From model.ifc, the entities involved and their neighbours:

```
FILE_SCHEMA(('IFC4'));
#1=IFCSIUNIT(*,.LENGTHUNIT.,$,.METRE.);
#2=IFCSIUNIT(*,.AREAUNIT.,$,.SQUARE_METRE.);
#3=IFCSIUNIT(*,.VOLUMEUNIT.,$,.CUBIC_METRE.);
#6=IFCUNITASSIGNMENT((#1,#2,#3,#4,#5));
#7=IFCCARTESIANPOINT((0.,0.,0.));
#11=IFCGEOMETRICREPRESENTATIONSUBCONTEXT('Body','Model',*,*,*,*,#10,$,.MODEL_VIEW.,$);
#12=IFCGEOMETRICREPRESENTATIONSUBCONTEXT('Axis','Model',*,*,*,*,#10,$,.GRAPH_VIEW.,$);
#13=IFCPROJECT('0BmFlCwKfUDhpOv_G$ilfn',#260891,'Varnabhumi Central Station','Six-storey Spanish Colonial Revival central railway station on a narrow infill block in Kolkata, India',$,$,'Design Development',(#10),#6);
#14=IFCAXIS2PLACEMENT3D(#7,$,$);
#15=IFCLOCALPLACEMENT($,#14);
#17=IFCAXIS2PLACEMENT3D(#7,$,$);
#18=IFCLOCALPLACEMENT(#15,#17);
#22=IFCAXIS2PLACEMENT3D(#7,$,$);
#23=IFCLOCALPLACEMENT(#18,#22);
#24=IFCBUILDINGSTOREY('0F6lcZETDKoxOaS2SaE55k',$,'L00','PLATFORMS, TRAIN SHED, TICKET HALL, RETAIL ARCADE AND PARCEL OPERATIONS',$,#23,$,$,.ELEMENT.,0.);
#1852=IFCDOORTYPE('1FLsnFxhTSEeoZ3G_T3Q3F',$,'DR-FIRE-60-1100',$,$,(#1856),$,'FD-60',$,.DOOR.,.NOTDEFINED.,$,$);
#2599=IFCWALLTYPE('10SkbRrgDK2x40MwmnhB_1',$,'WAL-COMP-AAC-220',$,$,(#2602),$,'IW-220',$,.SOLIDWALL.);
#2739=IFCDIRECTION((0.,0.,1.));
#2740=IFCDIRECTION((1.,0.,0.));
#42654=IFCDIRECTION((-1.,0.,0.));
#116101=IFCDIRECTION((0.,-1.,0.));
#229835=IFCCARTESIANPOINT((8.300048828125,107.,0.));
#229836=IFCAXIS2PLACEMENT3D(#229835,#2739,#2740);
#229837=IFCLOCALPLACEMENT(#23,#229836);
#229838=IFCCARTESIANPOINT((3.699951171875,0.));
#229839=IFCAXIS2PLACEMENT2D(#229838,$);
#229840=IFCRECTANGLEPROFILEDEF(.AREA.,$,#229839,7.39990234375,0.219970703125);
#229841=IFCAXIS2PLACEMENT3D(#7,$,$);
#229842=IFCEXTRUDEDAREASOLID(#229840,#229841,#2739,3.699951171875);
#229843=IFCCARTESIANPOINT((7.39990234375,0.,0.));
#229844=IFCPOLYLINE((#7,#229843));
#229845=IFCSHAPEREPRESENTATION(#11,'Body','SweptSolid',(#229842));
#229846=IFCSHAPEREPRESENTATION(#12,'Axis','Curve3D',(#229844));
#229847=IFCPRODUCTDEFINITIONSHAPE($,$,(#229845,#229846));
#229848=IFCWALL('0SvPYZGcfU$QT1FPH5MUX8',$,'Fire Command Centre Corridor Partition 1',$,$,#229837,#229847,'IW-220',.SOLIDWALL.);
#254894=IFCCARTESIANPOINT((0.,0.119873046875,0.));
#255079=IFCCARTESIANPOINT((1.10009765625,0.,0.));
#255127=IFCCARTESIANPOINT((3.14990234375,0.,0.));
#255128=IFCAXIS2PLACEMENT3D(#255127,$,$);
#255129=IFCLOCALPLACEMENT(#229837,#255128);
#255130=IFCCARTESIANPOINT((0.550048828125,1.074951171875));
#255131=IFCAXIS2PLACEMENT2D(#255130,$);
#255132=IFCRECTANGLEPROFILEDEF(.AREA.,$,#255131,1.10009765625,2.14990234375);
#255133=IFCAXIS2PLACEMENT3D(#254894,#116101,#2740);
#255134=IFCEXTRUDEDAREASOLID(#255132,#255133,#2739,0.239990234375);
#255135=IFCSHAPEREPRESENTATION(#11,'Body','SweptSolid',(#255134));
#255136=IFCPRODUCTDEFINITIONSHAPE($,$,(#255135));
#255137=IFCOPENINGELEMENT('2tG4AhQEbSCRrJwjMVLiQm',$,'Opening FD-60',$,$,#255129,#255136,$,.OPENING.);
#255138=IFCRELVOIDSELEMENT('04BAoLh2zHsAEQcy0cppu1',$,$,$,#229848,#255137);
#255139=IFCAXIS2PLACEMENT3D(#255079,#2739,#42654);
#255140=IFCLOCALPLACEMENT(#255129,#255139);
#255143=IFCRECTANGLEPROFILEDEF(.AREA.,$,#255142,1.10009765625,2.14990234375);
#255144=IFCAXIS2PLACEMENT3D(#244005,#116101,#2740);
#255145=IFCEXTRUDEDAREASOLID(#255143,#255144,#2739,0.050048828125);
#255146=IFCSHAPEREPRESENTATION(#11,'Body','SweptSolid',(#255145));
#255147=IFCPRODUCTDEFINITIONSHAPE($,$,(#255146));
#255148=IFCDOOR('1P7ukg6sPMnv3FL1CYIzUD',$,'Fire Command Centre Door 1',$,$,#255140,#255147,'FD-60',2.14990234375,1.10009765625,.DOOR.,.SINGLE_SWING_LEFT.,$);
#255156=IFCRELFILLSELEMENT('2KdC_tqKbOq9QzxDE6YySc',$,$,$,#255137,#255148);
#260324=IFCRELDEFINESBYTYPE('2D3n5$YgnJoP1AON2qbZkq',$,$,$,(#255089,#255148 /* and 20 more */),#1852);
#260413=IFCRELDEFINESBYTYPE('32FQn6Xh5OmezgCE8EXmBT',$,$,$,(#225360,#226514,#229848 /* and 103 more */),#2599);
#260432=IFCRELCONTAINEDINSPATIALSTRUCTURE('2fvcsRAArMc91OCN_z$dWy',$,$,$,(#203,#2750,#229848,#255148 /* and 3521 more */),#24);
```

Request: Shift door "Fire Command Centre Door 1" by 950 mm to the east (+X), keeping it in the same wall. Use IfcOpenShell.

```python
import ifcopenshell
import ifcopenshell.api.geometry
import ifcopenshell.util.placement
import ifcopenshell.util.unit

model = ifcopenshell.open("model.ifc")
unit_scale = ifcopenshell.util.unit.calculate_unit_scale(model)

door = model.by_guid("1P7ukg6sPMnv3FL1CYIzUD")
opening = door.FillsVoids[0].RelatingOpeningElement
wall = opening.VoidsElements[0].RelatingBuildingElement

wall_matrix = ifcopenshell.util.placement.get_local_placement(wall.ObjectPlacement)
shift = wall_matrix[:3, 0] * 0.95 / unit_scale
before = ifcopenshell.util.placement.get_local_placement(door.ObjectPlacement)[:3, 3].copy()

# The door is placed relative to its opening, so it follows when the opening moves.
matrix = ifcopenshell.util.placement.get_local_placement(opening.ObjectPlacement)
matrix[:3, 3] += shift
ifcopenshell.api.geometry.edit_object_placement(
    model, product=opening, matrix=matrix, is_si=False, should_transform_children=True
)

after = ifcopenshell.util.placement.get_local_placement(door.ObjectPlacement)[:3, 3]
print("door moved by", (after - before).round(3) + 0.0)

model.write("model-out.ifc")
```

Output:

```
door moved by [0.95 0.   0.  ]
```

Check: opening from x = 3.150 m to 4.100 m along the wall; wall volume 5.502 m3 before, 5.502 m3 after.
